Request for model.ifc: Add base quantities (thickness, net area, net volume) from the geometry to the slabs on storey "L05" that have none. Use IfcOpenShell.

First a look at what the model holds.

```python
import ifcopenshell
import ifcopenshell.util.element
import ifcopenshell.util.unit

model = ifcopenshell.open("model.ifc")
print(model.schema)
for unit_type in ("LENGTHUNIT", "AREAUNIT", "VOLUMEUNIT"):
    print(unit_type, ifcopenshell.util.unit.calculate_unit_scale(model, unit_type))
storey = next(s for s in model.by_type("IfcBuildingStorey") if s.Name == "L05")
slabs = [e for e in ifcopenshell.util.element.get_decomposition(storey) if e.is_a("IfcSlab")]
for e in sorted(slabs, key=lambda e: e.id()):
    print(e.id(), e.is_a(), e.Name, list(ifcopenshell.util.element.get_psets(e, qtos_only=True)), sep=" | ")
```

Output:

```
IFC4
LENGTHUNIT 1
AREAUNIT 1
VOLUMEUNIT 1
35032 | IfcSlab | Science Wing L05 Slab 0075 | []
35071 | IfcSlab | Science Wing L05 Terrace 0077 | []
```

```python
import ifcopenshell
import ifcopenshell.api.pset
import ifcopenshell.geom
import ifcopenshell.util.element
import ifcopenshell.util.shape
import ifcopenshell.util.unit

model = ifcopenshell.open("model.ifc")
unit_scale = ifcopenshell.util.unit.calculate_unit_scale(model)
area_scale = ifcopenshell.util.unit.calculate_unit_scale(model, "AREAUNIT")
volume_scale = ifcopenshell.util.unit.calculate_unit_scale(model, "VOLUMEUNIT")
settings = ifcopenshell.geom.settings()

storey = next(s for s in model.by_type("IfcBuildingStorey") if s.Name == "L05")
slabs = [e for e in ifcopenshell.util.element.get_decomposition(storey) if e.is_a("IfcSlab")]

for e in sorted(slabs, key=lambda e: e.id()):
    if ifcopenshell.util.element.get_psets(e, qtos_only=True, should_inherit=False):
        continue
    # Geometry comes back in metres, in the element's own axes.
    shape = ifcopenshell.geom.create_shape(settings, e)
    values = {
        "Width": ifcopenshell.util.shape.get_z(shape.geometry) / unit_scale,
        "NetArea": ifcopenshell.util.shape.get_footprint_area(shape.geometry) / area_scale,
        "NetVolume": ifcopenshell.util.shape.get_volume(shape.geometry) / volume_scale,
    }
    qto = ifcopenshell.api.pset.add_qto(model, product=e, name="Qto_SlabBaseQuantities")
    ifcopenshell.api.pset.edit_qto(model, qto=qto, properties=values)
    print(e.id(), {k: round(v, 3) for k, v in values.items()})

model.write("model-out.ifc")
```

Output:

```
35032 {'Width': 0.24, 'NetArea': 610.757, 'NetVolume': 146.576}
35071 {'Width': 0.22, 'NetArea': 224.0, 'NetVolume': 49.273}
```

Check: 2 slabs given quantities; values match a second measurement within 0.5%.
